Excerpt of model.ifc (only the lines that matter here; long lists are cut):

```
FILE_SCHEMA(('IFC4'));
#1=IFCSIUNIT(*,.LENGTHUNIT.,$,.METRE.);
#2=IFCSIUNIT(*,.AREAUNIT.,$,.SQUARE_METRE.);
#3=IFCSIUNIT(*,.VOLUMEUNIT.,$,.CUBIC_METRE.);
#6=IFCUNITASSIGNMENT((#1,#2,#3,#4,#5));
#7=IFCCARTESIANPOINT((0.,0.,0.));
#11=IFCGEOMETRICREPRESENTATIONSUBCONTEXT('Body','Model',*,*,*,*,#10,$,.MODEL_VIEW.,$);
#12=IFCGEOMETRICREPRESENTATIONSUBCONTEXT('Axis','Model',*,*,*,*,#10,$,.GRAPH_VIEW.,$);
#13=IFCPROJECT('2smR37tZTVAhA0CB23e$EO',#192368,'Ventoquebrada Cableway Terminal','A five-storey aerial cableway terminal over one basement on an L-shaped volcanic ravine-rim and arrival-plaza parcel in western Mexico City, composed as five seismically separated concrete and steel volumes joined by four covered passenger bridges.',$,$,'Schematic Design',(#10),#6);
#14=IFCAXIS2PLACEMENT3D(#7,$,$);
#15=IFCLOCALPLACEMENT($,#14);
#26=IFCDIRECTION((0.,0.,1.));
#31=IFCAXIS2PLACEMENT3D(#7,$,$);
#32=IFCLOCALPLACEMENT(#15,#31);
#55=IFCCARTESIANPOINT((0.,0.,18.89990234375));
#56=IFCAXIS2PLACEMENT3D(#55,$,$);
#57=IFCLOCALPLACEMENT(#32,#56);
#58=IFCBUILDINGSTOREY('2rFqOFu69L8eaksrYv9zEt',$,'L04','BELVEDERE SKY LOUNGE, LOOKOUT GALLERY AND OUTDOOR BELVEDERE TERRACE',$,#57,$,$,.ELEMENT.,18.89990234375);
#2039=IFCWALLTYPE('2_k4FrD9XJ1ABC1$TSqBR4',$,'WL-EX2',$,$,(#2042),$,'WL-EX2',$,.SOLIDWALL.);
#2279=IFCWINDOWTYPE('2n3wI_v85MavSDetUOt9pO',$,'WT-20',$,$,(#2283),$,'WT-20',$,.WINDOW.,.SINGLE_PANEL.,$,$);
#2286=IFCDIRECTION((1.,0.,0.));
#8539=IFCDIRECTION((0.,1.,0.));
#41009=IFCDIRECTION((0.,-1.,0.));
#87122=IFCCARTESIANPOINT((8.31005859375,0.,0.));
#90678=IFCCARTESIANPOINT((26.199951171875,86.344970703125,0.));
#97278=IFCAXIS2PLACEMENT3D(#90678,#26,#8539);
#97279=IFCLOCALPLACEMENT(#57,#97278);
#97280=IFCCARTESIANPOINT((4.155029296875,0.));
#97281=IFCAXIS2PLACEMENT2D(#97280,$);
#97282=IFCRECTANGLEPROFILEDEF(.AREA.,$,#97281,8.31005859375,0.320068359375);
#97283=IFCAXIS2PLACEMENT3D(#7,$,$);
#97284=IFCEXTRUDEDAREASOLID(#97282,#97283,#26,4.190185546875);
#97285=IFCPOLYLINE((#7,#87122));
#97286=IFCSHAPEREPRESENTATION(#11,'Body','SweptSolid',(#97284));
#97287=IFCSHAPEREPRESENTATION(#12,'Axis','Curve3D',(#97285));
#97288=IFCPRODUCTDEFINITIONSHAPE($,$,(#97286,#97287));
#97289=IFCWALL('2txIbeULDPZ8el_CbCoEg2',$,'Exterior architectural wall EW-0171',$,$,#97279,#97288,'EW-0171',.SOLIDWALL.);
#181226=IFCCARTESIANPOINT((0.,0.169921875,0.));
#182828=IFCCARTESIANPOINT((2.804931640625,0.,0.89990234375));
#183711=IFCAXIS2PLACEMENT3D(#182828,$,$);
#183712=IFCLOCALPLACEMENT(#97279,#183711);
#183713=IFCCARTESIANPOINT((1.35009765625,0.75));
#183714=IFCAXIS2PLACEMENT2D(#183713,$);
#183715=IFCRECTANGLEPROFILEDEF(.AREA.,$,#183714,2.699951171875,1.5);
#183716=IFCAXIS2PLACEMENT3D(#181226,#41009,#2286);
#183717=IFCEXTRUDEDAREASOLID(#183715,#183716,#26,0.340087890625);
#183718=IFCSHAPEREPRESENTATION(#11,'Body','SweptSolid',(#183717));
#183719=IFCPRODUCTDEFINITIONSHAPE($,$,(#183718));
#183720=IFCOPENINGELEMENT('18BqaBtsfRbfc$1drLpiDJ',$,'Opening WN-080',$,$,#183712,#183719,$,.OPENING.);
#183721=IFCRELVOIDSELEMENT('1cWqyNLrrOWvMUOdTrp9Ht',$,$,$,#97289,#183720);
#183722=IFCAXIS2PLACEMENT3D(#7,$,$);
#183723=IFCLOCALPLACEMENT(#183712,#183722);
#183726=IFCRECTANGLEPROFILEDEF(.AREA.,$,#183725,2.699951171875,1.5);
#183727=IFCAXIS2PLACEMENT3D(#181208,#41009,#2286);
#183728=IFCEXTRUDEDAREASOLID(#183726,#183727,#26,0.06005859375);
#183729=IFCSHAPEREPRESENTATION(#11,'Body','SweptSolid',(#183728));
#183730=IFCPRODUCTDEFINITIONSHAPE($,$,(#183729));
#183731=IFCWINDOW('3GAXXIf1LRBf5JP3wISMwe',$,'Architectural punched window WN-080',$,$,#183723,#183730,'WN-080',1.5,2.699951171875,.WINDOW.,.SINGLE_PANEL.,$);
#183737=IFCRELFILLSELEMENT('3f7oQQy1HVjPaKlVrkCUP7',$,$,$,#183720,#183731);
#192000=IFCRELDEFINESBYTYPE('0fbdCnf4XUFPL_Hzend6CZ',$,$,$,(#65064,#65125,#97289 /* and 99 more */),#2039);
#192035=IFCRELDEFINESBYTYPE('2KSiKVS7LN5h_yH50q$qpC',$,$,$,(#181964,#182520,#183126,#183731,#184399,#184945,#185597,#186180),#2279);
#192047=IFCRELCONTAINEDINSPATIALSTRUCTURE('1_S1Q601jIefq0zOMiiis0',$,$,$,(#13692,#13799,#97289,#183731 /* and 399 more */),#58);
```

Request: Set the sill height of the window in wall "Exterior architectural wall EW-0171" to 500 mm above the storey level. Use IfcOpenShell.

```python
import numpy as np
import ifcopenshell
import ifcopenshell.api.geometry
import ifcopenshell.geom
import ifcopenshell.util.element
import ifcopenshell.util.placement
import ifcopenshell.util.shape
import ifcopenshell.util.unit

model = ifcopenshell.open("model.ifc")
unit_scale = ifcopenshell.util.unit.calculate_unit_scale(model)

window = model.by_guid("3GAXXIf1LRBf5JP3wISMwe")
opening = window.FillsVoids[0].RelatingOpeningElement
storey = ifcopenshell.util.element.get_container(window, ifc_class="IfcBuildingStorey")
level = ifcopenshell.util.placement.get_local_placement(storey.ObjectPlacement)[2, 3]

# The opening's origin need not be at the sill, so measure its lowest point.
shape = ifcopenshell.geom.create_shape(ifcopenshell.geom.settings(), opening)
bottom = ifcopenshell.util.shape.get_shape_bottom_elevation(shape, shape.geometry) / unit_scale
dz = level + 0.5 - bottom

shift = np.array([0.0, 0.0, dz])
# The window is placed relative to its opening, so it follows when the opening moves.
matrix = ifcopenshell.util.placement.get_local_placement(opening.ObjectPlacement)
matrix[:3, 3] += shift
ifcopenshell.api.geometry.edit_object_placement(
    model, product=opening, matrix=matrix, is_si=False, should_transform_children=True
)

print(f"moved by {dz * unit_scale:+.3f} m")

model.write("model-out.ifc")
```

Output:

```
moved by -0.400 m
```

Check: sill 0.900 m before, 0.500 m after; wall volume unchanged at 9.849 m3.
